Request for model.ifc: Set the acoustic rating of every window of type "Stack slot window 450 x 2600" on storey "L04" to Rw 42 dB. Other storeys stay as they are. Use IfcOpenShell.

First a look at what the model holds.

```python
import ifcopenshell
import ifcopenshell.util.element

model = ifcopenshell.open("model.ifc")
print(model.schema)
storey = next(s for s in model.by_type("IfcBuildingStorey") if s.Name == "L04")
windows = [e for e in ifcopenshell.util.element.get_decomposition(storey) if e.is_a("IfcWindow")]
seen = {}
for e in windows:
    element_type = ifcopenshell.util.element.get_type(e)
    key = (element_type.Name if element_type != e and element_type else None, ifcopenshell.util.element.get_pset(e, "Pset_WindowCommon", "AcousticRating"))
    seen[key] = seen.get(key, 0) + 1
for (name, value), count in sorted(seen.items(), key=str):
    print(count, "x", name, "|", value)
```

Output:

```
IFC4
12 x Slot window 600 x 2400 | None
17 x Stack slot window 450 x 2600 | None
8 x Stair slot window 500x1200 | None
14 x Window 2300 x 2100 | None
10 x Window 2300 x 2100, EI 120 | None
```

```python
import ifcopenshell
import ifcopenshell.api.pset
import ifcopenshell.util.element

model = ifcopenshell.open("model.ifc")

storey = next(s for s in model.by_type("IfcBuildingStorey") if s.Name == "L04")
windows = [e for e in ifcopenshell.util.element.get_decomposition(storey) if e.is_a("IfcWindow")]

count = 0
for e in windows:
    element_type = ifcopenshell.util.element.get_type(e)
    if element_type in (None, e) or element_type.Name != "Stack slot window 450 x 2600":
        continue
    # add_pset returns the element's existing set when there is one.
    pset = ifcopenshell.api.pset.add_pset(model, product=e, name="Pset_WindowCommon")
    ifcopenshell.api.pset.edit_pset(model, pset=pset, properties={"AcousticRating": "Rw 42 dB"})
    count += 1

print(count, "windows updated")

model.write("model_edited.ifc")
```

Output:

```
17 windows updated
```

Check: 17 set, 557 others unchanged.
